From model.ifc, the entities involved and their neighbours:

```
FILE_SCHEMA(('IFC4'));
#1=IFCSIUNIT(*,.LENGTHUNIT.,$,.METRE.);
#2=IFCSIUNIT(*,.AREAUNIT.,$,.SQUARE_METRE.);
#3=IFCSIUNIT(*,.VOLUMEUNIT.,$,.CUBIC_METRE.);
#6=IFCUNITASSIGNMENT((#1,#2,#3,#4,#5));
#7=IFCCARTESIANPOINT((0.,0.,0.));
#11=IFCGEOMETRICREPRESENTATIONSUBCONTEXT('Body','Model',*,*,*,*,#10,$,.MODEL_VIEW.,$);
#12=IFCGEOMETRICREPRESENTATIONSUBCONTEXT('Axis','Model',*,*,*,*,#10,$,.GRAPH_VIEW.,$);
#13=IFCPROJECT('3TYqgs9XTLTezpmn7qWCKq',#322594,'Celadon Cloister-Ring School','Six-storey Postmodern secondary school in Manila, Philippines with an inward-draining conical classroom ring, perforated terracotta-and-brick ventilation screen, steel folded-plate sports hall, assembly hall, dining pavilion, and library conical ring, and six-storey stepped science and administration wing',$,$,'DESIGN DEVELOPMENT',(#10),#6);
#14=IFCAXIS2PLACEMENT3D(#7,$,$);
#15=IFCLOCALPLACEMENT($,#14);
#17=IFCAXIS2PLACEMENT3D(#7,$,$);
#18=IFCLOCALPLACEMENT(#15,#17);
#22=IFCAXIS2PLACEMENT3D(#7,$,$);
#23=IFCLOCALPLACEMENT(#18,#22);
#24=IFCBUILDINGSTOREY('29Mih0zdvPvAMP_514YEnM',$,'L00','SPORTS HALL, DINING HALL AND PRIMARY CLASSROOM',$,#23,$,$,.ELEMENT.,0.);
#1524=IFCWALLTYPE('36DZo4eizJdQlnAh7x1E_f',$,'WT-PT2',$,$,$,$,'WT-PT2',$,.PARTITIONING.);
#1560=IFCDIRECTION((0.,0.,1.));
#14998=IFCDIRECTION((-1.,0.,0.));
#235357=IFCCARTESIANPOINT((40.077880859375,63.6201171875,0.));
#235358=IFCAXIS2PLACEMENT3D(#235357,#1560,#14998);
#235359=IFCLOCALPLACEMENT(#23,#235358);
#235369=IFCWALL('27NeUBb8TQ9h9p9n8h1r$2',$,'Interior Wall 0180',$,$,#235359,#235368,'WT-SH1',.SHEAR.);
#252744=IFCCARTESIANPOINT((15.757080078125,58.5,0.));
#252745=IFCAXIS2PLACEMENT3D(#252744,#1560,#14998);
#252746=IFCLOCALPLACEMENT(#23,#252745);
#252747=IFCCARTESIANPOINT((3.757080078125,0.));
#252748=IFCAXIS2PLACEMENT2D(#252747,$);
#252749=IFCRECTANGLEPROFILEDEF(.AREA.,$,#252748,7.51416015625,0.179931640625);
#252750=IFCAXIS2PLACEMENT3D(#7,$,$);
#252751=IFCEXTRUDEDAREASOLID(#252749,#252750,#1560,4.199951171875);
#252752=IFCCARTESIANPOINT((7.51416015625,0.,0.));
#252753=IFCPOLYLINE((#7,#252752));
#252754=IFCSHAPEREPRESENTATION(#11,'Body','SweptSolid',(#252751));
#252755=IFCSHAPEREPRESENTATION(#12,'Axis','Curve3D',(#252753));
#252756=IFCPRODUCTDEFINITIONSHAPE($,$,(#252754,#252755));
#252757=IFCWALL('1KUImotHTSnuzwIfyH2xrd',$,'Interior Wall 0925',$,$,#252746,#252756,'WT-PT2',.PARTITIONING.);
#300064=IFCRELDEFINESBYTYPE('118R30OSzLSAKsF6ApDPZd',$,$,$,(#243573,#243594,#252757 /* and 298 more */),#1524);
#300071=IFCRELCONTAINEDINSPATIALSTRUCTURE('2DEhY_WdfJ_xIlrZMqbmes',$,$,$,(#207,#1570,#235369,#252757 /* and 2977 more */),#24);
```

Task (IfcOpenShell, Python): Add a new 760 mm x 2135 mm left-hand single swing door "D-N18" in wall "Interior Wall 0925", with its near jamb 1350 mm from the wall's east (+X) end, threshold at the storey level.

```python
import numpy as np
import ifcopenshell
import ifcopenshell.api.feature
import ifcopenshell.api.geometry
import ifcopenshell.api.root
import ifcopenshell.api.spatial
import ifcopenshell.geom
import ifcopenshell.util.element
import ifcopenshell.util.placement
import ifcopenshell.util.representation
import ifcopenshell.util.shape
import ifcopenshell.util.unit

model = ifcopenshell.open("model.ifc")
unit_scale = ifcopenshell.util.unit.calculate_unit_scale(model)
settings = ifcopenshell.geom.settings()


def volume(element):
    """Net volume in cubic metres, openings subtracted."""
    shape = ifcopenshell.geom.create_shape(settings, element)
    return ifcopenshell.util.shape.get_volume(shape.geometry)


wall = model.by_id(252757)
storey = ifcopenshell.util.element.get_container(wall, ifc_class="IfcBuildingStorey")
context = ifcopenshell.util.representation.get_context(model, "Model", "Body", "MODEL_VIEW")
before = volume(wall)

width, height, from_end, sill = 0.76, 2.135, 1.35, 0.0  # metres

# The wall runs along its own X axis, and the end named is its -X end.
wall_shape = ifcopenshell.geom.create_shape(settings, wall)
x, y, z = ifcopenshell.util.shape.get_vertices(wall_shape.geometry).T
start = x.min() + from_end
face, thickness = float(y.min()), float(y.max() - y.min())
wall_matrix = ifcopenshell.util.placement.get_local_placement(wall.ObjectPlacement)
level = ifcopenshell.util.placement.get_local_placement(storey.ObjectPlacement)[2, 3]


def in_wall(x, y):
    """Placement at x, y metres in the wall's axes, at sill height."""
    matrix = wall_matrix.copy()
    matrix[:, 3] = wall_matrix @ np.array([x / unit_scale, y / unit_scale, 0.0, 1.0])
    matrix[2, 3] = level + sill / unit_scale
    return matrix


# Opening: a box that overshoots both wall faces by 50 mm.
opening = ifcopenshell.api.root.create_entity(model, ifc_class="IfcOpeningElement", predefined_type="OPENING")
box = ifcopenshell.api.geometry.add_wall_representation(
    model, context=context, length=width, height=height, thickness=thickness + 0.1
)
ifcopenshell.api.geometry.assign_representation(model, product=opening, representation=box)
ifcopenshell.api.geometry.edit_object_placement(model, product=opening, matrix=in_wall(start, face - 0.05), is_si=False)
ifcopenshell.api.feature.add_feature(model, feature=opening, element=wall)

door = ifcopenshell.api.root.create_entity(model, ifc_class="IfcDoor", name="D-N18", predefined_type="DOOR")
door.OverallWidth, door.OverallHeight = width / unit_scale, height / unit_scale
door.OperationType = "SINGLE_SWING_LEFT"
body = ifcopenshell.api.geometry.add_door_representation(
    model,
    context=context,
    overall_width=door.OverallWidth,
    overall_height=door.OverallHeight,
    operation_type="SINGLE_SWING_LEFT",
    lining_properties={"LiningDepth": thickness / unit_scale, "ThresholdDepth": thickness / unit_scale},
)
ifcopenshell.api.geometry.assign_representation(model, product=door, representation=body)
ifcopenshell.api.spatial.assign_container(model, products=[door], relating_structure=storey)
ifcopenshell.api.feature.add_filling(model, opening=opening, element=door)

# The lining spans the wall, so the door starts at the wall face.
ifcopenshell.api.geometry.edit_object_placement(model, product=door, matrix=in_wall(start, face), is_si=False)

after = volume(wall)

print(f"wall volume {before:.3f} -> {after:.3f} m3")

model.write("model_v2.ifc")
```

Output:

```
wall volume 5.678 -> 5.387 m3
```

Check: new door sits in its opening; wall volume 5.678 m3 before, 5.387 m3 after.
